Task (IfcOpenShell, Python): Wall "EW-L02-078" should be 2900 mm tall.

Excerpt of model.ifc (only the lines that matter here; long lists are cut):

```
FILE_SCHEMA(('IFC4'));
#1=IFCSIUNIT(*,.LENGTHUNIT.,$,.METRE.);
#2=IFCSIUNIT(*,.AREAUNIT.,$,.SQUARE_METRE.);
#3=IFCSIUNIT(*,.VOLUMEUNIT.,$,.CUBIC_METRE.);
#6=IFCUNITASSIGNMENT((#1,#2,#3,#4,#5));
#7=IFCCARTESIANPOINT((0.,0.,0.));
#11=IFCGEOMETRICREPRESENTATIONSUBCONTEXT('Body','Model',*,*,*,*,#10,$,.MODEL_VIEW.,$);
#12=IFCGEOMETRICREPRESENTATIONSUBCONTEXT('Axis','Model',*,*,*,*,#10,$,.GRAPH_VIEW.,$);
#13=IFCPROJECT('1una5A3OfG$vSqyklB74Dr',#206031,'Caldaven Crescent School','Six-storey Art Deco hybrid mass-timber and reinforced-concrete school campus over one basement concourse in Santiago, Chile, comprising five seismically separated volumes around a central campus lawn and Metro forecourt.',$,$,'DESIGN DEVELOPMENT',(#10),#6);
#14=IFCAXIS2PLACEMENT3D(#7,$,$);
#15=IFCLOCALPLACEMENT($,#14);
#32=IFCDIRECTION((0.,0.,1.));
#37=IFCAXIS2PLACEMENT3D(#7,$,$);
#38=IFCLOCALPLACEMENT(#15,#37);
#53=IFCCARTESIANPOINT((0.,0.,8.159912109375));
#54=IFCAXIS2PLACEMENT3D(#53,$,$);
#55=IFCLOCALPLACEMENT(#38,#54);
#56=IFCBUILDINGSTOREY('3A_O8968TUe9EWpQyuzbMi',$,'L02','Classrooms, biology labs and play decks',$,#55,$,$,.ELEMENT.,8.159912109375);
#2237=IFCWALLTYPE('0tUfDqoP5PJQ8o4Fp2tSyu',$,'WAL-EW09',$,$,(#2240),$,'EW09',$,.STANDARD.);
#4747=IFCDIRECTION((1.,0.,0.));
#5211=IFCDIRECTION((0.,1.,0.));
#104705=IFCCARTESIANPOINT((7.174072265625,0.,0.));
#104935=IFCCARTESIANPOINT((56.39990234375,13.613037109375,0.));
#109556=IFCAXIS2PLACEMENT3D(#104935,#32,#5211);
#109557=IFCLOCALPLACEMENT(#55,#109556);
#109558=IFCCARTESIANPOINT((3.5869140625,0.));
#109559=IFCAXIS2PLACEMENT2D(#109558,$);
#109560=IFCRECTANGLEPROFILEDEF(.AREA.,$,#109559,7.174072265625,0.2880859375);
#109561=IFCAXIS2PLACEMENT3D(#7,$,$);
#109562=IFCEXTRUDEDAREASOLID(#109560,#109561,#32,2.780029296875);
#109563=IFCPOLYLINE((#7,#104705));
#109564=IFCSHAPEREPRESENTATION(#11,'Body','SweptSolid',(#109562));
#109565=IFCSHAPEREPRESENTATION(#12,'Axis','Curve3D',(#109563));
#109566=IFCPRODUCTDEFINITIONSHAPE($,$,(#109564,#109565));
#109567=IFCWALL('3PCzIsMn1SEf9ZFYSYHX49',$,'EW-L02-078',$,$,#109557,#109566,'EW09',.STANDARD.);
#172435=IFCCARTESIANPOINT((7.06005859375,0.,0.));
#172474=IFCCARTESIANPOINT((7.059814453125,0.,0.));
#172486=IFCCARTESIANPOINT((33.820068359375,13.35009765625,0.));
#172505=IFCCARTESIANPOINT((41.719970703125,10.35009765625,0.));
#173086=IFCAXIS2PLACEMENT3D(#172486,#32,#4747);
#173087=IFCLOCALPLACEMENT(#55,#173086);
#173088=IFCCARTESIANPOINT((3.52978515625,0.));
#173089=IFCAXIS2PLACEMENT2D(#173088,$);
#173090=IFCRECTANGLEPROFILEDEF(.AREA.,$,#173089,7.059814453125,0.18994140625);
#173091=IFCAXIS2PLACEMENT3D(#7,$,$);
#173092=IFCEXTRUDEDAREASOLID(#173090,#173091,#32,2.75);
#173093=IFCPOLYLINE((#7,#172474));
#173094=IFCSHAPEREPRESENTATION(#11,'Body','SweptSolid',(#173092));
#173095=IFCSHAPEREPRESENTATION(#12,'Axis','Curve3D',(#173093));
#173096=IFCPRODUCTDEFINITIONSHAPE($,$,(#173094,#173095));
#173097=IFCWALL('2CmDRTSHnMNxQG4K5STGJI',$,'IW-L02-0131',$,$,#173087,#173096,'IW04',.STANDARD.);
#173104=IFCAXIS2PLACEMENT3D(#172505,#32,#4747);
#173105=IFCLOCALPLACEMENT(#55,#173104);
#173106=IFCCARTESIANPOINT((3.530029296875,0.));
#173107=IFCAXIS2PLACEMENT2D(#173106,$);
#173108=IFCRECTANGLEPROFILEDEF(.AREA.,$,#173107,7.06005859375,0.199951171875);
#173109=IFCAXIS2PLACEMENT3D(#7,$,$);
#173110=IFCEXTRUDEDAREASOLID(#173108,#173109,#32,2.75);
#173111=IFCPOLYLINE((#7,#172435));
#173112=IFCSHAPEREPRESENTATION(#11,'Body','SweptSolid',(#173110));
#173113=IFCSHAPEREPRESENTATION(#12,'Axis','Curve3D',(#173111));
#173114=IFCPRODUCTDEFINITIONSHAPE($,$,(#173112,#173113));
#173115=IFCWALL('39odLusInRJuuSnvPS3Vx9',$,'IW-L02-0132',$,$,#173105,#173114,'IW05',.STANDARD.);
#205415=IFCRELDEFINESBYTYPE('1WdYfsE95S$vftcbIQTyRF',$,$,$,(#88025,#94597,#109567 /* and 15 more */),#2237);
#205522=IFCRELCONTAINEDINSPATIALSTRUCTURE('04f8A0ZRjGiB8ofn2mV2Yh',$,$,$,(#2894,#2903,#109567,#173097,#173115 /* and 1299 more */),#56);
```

```python
import ifcopenshell
import ifcopenshell.geom
import ifcopenshell.util.representation
import ifcopenshell.util.shape
import ifcopenshell.util.unit

model = ifcopenshell.open("model.ifc")
unit_scale = ifcopenshell.util.unit.calculate_unit_scale(model)
settings = ifcopenshell.geom.settings()


def volume(element):
    """Net volume in cubic metres, openings subtracted."""
    shape = ifcopenshell.geom.create_shape(settings, element)
    return ifcopenshell.util.shape.get_volume(shape.geometry)


wall = model.by_guid("3PCzIsMn1SEf9ZFYSYHX49")
before = volume(wall)

body = ifcopenshell.util.representation.get_representation(wall, "Model", "Body")
solid = body.Items[0]
old_height = solid.Depth
solid.Depth = 2.9 / unit_scale
after = volume(wall)

print(f"height {old_height:g} -> {solid.Depth:g}, volume {before:.3f} -> {after:.3f} m3")

model.write("model_updated.ifc")
```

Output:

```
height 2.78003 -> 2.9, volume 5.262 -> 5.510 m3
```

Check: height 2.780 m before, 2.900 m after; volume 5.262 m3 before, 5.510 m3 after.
